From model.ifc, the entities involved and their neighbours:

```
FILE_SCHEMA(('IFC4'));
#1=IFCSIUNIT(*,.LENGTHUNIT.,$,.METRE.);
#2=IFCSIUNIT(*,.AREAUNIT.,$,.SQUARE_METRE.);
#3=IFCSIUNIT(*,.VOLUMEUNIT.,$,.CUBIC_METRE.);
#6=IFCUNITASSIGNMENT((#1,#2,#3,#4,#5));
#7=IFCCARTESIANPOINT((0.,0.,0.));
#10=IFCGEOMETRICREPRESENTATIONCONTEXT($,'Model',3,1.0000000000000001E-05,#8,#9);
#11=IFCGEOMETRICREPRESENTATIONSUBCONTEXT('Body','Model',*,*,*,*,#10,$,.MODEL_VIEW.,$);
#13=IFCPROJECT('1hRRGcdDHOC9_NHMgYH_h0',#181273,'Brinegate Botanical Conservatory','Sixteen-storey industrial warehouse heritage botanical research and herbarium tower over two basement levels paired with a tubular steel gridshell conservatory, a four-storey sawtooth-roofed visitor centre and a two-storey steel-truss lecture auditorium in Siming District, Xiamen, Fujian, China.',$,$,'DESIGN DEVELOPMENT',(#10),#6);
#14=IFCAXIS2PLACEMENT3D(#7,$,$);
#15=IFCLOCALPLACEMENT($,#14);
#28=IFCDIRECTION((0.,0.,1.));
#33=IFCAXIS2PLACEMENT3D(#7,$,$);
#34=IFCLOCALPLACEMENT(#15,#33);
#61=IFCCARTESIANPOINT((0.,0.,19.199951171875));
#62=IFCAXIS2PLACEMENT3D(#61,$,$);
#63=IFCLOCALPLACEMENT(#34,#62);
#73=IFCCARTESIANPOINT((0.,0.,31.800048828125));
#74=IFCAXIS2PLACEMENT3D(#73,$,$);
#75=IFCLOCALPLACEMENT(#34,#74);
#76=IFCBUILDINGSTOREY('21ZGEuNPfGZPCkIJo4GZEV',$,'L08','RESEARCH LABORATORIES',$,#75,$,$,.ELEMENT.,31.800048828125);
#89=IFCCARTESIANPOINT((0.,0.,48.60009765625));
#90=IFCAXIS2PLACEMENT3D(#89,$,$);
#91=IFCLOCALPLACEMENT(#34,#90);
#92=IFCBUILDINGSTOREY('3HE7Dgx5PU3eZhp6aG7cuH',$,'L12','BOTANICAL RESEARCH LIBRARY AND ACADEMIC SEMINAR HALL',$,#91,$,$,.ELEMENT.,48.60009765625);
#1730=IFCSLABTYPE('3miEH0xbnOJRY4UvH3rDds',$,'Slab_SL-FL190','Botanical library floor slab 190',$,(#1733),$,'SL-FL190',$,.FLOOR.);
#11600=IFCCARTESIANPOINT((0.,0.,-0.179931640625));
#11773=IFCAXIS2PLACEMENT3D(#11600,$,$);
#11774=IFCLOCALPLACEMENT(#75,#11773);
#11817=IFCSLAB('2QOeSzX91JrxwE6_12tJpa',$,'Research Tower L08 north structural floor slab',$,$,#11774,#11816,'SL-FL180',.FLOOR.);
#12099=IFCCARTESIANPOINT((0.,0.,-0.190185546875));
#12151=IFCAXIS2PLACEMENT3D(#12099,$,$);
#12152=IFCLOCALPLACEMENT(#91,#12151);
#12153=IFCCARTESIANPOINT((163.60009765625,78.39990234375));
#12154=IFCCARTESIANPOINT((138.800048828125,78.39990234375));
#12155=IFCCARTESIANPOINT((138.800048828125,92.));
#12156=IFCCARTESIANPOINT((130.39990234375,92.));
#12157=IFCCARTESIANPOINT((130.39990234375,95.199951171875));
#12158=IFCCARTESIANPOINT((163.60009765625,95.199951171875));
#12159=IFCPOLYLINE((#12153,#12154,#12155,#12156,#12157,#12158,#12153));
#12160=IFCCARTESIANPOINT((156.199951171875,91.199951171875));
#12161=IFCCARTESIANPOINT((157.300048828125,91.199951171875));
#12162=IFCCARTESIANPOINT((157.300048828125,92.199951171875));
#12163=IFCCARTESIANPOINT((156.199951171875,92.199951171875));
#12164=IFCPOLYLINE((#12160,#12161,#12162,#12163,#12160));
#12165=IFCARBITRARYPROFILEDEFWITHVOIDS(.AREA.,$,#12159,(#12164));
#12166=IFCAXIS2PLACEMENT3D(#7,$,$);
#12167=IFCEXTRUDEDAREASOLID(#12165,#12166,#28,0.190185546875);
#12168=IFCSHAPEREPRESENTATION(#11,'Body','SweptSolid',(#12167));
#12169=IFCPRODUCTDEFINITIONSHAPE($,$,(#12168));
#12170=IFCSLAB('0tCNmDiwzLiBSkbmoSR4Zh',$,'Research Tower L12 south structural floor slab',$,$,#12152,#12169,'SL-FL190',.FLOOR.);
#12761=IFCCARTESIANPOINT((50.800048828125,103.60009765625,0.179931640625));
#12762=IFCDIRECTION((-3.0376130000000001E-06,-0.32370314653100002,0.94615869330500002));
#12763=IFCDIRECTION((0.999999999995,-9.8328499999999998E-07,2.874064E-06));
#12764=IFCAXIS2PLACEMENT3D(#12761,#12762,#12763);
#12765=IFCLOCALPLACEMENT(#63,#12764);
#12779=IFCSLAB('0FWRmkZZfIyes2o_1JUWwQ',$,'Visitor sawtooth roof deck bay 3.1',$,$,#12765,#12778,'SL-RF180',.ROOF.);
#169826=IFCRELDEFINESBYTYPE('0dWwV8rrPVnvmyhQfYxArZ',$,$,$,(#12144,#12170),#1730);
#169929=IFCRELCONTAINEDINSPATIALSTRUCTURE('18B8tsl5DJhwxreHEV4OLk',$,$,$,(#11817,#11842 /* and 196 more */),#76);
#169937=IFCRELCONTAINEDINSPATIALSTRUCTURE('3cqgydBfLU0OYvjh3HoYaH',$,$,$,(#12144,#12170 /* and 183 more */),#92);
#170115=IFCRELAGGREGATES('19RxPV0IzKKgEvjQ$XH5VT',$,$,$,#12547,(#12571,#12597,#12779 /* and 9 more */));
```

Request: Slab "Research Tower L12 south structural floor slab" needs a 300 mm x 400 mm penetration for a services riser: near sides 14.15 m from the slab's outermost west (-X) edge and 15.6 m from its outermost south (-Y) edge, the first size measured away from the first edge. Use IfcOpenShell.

```python
import numpy as np
import ifcopenshell
import ifcopenshell.api.feature
import ifcopenshell.api.geometry
import ifcopenshell.api.root
import ifcopenshell.geom
import ifcopenshell.util.placement
import ifcopenshell.util.representation
import ifcopenshell.util.shape
import ifcopenshell.util.unit

model = ifcopenshell.open("model.ifc")
unit_scale = ifcopenshell.util.unit.calculate_unit_scale(model)
settings = ifcopenshell.geom.settings()


def volume(element):
    """Net volume in cubic metres, openings subtracted."""
    shape = ifcopenshell.geom.create_shape(settings, element)
    return ifcopenshell.util.shape.get_volume(shape.geometry)


slab = model.by_id(12170)
before = volume(slab)

# Extent in the slab's own axes, in metres. The edges named are its -X and -Y sides.
slab_shape = ifcopenshell.geom.create_shape(settings, slab)
vertices = ifcopenshell.util.shape.get_vertices(slab_shape.geometry)
x_min, y_min, bottom = vertices.min(axis=0)
top = vertices[:, 2].max()

opening = ifcopenshell.api.root.create_entity(model, ifc_class="IfcOpeningElement", name="Services riser opening", predefined_type="OPENING")
context = ifcopenshell.util.representation.get_context(model, "Model", "Body", "MODEL_VIEW")
width, depth = 0.3, 0.4
outline = [(0.0, 0.0), (width, 0.0), (width, depth), (0.0, depth), (0.0, 0.0)]
# Overshoot both faces by 50 mm so the cut is clean.
shape = ifcopenshell.api.geometry.add_slab_representation(
    model, context=context, depth=top - bottom + 0.1, polyline=outline
)
ifcopenshell.api.geometry.assign_representation(model, product=opening, representation=shape)

matrix = ifcopenshell.util.placement.get_local_placement(slab.ObjectPlacement)
matrix[:, 3] = matrix @ np.append(np.array([x_min + 14.15, y_min + 15.6, bottom - 0.05]) / unit_scale, 1.0)
ifcopenshell.api.geometry.edit_object_placement(model, product=opening, matrix=matrix, is_si=False)
ifcopenshell.api.feature.add_feature(model, feature=opening, element=slab)

after = volume(slab)

print(f"slab volume {before:.3f} -> {after:.3f} m3")

model.write("model_rev.ifc")
```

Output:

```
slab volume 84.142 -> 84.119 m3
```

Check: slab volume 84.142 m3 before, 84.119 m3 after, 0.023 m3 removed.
